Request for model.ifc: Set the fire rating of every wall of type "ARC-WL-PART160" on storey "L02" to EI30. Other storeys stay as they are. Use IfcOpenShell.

First a look at what the model holds.

```python
import ifcopenshell
import ifcopenshell.util.element

model = ifcopenshell.open("model.ifc")
print(model.schema)
storey = next(s for s in model.by_type("IfcBuildingStorey") if s.Name == "L02")
walls = [e for e in ifcopenshell.util.element.get_decomposition(storey) if e.is_a("IfcWall")]
seen = {}
for e in walls:
    element_type = ifcopenshell.util.element.get_type(e)
    key = (element_type.Name if element_type != e and element_type else None, ifcopenshell.util.element.get_pset(e, "Pset_WallCommon", "FireRating"))
    seen[key] = seen.get(key, 0) + 1
for (name, value), count in sorted(seen.items(), key=str):
    print(count, "x", name, "|", value)
```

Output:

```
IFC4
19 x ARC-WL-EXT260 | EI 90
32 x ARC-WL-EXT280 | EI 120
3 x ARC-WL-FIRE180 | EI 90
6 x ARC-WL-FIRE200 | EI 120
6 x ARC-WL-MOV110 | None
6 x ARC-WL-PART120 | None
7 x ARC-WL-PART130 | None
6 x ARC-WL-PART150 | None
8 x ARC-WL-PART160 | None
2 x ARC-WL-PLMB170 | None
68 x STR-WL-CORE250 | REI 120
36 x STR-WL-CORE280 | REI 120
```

```python
import ifcopenshell
import ifcopenshell.api.pset
import ifcopenshell.util.element

model = ifcopenshell.open("model.ifc")

storey = next(s for s in model.by_type("IfcBuildingStorey") if s.Name == "L02")
walls = [e for e in ifcopenshell.util.element.get_decomposition(storey) if e.is_a("IfcWall")]

count = 0
for e in walls:
    element_type = ifcopenshell.util.element.get_type(e)
    if element_type in (None, e) or element_type.Name != "ARC-WL-PART160":
        continue
    # add_pset returns the element's existing set when there is one.
    pset = ifcopenshell.api.pset.add_pset(model, product=e, name="Pset_WallCommon")
    ifcopenshell.api.pset.edit_pset(model, pset=pset, properties={"FireRating": "EI30"})
    count += 1

print(count, "walls updated")

model.write("model-out.ifc")
```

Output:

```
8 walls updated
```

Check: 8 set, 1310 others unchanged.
